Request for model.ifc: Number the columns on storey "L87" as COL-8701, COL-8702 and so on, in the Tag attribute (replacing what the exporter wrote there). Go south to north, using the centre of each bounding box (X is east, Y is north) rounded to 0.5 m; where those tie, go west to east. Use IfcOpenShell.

First a look at what the model holds.

```python
import ifcopenshell
import ifcopenshell.util.element
import ifcopenshell.util.placement

model = ifcopenshell.open("model.ifc")
print(model.schema)
storey = next(s for s in model.by_type("IfcBuildingStorey") if s.Name == "L87")
columns = [e for e in ifcopenshell.util.element.get_decomposition(storey) if e.is_a("IfcColumn")]
for e in sorted(columns, key=lambda e: e.id()):
    origin = ifcopenshell.util.placement.get_local_placement(e.ObjectPlacement)[:3, 3]
    print(e.id(), e.Tag, e.Name, origin.round(2) + 0.0, sep=" | ")
```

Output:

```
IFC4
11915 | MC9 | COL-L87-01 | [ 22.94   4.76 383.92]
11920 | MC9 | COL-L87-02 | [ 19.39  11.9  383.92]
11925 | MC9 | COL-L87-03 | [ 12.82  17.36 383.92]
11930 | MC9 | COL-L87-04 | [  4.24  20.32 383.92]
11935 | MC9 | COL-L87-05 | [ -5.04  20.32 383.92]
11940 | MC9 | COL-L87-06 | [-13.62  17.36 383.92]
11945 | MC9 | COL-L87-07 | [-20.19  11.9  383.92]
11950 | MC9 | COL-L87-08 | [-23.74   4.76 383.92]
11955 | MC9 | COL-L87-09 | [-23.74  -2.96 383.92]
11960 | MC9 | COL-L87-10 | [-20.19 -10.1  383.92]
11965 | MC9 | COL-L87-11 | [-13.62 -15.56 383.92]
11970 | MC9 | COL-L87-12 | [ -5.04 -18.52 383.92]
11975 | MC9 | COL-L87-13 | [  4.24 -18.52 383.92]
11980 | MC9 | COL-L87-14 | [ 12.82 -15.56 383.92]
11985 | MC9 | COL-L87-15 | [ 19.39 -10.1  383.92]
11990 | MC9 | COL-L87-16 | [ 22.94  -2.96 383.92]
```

```python
import ifcopenshell
import ifcopenshell.geom
import ifcopenshell.util.element
import ifcopenshell.util.shape

model = ifcopenshell.open("model.ifc")
settings = ifcopenshell.geom.settings()
settings.set("use-world-coords", True)


def centre(element):
    shape = ifcopenshell.geom.create_shape(settings, element)
    return ifcopenshell.util.shape.get_bbox_centroid(shape.geometry)


storey = next(s for s in model.by_type("IfcBuildingStorey") if s.Name == "L87")
columns = [e for e in ifcopenshell.util.element.get_decomposition(storey) if e.is_a("IfcColumn")]

# Insertion points can sit at a corner or the storey origin, so sort by the geometry (in metres).
centres = {e: centre(e) for e in columns}
columns.sort(key=lambda e: (round(centres[e][1] / 0.5), centres[e][0]))

for i, e in enumerate(columns, start=1):
    number = f"COL-87{i:02d}"
    e.Tag = number
    print(e.id(), number)

model.write("model_rev.ifc")
```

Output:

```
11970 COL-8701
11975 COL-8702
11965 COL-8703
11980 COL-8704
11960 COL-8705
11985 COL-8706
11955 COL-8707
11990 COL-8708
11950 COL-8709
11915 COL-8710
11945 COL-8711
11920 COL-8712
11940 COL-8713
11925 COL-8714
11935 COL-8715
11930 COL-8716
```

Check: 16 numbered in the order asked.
